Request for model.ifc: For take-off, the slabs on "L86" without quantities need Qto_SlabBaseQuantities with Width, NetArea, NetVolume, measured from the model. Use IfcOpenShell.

First a look at what the model holds.

```python
import ifcopenshell
import ifcopenshell.util.element
import ifcopenshell.util.unit

model = ifcopenshell.open("model.ifc")
print(model.schema)
for unit_type in ("LENGTHUNIT", "AREAUNIT", "VOLUMEUNIT"):
    print(unit_type, ifcopenshell.util.unit.calculate_unit_scale(model, unit_type))
storey = next(s for s in model.by_type("IfcBuildingStorey") if s.Name == "L86")
slabs = [e for e in ifcopenshell.util.element.get_decomposition(storey) if e.is_a("IfcSlab")]
for e in sorted(slabs, key=lambda e: e.id()):
    print(e.id(), e.is_a(), e.Name, list(ifcopenshell.util.element.get_psets(e, qtos_only=True)), sep=" | ")
```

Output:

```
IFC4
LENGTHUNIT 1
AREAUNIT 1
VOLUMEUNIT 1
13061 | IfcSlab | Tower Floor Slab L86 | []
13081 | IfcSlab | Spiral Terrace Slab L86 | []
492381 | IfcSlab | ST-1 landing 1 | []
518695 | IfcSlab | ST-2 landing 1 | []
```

```python
import ifcopenshell
import ifcopenshell.api.pset
import ifcopenshell.geom
import ifcopenshell.util.element
import ifcopenshell.util.shape
import ifcopenshell.util.unit

model = ifcopenshell.open("model.ifc")
unit_scale = ifcopenshell.util.unit.calculate_unit_scale(model)
area_scale = ifcopenshell.util.unit.calculate_unit_scale(model, "AREAUNIT")
volume_scale = ifcopenshell.util.unit.calculate_unit_scale(model, "VOLUMEUNIT")
settings = ifcopenshell.geom.settings()

storey = next(s for s in model.by_type("IfcBuildingStorey") if s.Name == "L86")
slabs = [e for e in ifcopenshell.util.element.get_decomposition(storey) if e.is_a("IfcSlab")]

for e in sorted(slabs, key=lambda e: e.id()):
    if ifcopenshell.util.element.get_psets(e, qtos_only=True, should_inherit=False):
        continue
    # Geometry comes back in metres, in the element's own axes.
    shape = ifcopenshell.geom.create_shape(settings, e)
    values = {
        "Width": ifcopenshell.util.shape.get_z(shape.geometry) / unit_scale,
        "NetArea": ifcopenshell.util.shape.get_footprint_area(shape.geometry) / area_scale,
        "NetVolume": ifcopenshell.util.shape.get_volume(shape.geometry) / volume_scale,
    }
    qto = ifcopenshell.api.pset.add_qto(model, product=e, name="Qto_SlabBaseQuantities")
    ifcopenshell.api.pset.edit_qto(model, qto=qto, properties=values)
    print(e.id(), {k: round(v, 3) for k, v in values.items()})

model.write("model_edited.ifc")
```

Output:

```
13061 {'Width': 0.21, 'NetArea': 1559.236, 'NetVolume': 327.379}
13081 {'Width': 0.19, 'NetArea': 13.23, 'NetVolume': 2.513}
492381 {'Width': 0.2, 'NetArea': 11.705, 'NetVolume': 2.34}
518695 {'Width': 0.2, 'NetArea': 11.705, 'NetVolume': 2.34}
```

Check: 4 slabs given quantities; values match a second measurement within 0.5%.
